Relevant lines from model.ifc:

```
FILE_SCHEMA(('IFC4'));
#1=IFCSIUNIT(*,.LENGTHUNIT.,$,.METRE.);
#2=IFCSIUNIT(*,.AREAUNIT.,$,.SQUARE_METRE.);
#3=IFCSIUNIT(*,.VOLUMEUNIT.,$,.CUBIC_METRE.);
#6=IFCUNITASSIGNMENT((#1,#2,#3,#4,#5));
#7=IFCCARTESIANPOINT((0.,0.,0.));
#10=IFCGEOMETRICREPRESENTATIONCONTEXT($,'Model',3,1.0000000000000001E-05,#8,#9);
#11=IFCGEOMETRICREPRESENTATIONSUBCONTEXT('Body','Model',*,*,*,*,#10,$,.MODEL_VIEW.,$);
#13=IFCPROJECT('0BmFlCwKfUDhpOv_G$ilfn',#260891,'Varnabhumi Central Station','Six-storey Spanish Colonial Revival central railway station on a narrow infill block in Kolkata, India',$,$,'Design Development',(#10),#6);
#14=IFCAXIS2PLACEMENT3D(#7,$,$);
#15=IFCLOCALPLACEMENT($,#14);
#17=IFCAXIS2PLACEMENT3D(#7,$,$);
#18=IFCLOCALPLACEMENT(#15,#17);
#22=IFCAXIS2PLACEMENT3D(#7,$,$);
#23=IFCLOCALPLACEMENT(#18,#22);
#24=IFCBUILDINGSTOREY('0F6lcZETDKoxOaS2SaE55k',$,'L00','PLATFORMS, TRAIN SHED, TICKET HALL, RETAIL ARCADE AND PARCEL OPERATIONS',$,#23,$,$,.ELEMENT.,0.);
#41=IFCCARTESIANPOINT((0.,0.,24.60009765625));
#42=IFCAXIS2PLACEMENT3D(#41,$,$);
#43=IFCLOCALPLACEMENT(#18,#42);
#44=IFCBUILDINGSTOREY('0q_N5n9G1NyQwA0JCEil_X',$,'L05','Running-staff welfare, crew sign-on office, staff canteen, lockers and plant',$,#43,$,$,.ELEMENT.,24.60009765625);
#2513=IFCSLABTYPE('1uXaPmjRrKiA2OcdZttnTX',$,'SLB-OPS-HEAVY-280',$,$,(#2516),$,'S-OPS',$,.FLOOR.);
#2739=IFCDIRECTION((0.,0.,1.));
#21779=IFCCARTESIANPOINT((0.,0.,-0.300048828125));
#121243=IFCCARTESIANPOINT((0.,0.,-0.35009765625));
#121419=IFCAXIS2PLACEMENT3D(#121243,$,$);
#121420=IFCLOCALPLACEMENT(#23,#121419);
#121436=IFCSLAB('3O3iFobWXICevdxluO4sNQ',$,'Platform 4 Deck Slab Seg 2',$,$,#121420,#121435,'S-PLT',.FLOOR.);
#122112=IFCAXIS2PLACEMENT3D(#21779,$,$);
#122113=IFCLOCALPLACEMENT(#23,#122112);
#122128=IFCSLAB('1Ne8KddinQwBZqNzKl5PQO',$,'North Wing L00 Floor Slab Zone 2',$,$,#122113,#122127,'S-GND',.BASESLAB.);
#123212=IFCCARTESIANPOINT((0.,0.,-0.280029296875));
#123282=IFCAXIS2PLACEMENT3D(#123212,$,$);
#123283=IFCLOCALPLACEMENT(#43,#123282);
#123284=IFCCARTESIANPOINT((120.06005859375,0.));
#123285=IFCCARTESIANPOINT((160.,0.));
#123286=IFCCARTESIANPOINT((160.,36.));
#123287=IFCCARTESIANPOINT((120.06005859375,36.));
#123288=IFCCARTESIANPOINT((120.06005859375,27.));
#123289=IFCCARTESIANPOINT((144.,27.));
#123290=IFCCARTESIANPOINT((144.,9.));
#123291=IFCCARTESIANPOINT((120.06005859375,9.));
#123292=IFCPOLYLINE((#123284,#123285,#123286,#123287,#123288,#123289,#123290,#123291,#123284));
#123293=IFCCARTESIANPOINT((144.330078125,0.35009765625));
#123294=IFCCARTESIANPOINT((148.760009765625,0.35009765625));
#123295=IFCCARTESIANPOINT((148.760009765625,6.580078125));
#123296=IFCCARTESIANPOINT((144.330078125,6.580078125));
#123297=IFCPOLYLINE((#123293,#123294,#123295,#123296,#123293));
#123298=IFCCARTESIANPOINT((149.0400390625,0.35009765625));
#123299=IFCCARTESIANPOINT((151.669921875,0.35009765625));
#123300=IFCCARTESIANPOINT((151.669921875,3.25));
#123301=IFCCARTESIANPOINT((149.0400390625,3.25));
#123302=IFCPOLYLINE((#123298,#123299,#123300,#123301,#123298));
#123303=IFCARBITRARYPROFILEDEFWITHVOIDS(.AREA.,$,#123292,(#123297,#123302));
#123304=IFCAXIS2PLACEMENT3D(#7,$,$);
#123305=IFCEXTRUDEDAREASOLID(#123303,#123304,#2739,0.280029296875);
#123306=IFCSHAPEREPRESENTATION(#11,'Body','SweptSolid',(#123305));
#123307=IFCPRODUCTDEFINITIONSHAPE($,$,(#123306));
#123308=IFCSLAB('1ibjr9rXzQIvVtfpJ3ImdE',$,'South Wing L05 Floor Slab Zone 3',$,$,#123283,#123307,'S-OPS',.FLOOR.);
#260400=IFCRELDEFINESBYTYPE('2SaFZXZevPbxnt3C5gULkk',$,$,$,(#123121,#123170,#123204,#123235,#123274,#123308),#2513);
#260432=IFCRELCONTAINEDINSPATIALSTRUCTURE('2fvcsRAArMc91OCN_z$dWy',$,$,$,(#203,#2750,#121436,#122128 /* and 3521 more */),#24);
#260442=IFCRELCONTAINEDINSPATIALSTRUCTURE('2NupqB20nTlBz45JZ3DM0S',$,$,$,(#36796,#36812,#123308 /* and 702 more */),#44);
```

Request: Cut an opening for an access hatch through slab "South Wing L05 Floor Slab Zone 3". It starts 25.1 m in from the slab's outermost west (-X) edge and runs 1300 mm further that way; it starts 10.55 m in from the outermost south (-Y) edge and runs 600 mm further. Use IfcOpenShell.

```python
import numpy as np
import ifcopenshell
import ifcopenshell.api.feature
import ifcopenshell.api.geometry
import ifcopenshell.api.root
import ifcopenshell.geom
import ifcopenshell.util.placement
import ifcopenshell.util.representation
import ifcopenshell.util.shape
import ifcopenshell.util.unit

model = ifcopenshell.open("model.ifc")
unit_scale = ifcopenshell.util.unit.calculate_unit_scale(model)
settings = ifcopenshell.geom.settings()


def volume(element):
    """Net volume in cubic metres, openings subtracted."""
    shape = ifcopenshell.geom.create_shape(settings, element)
    return ifcopenshell.util.shape.get_volume(shape.geometry)


slab = model.by_guid("1ibjr9rXzQIvVtfpJ3ImdE")
before = volume(slab)

# Extent in the slab's own axes, in metres. The edges named are its -X and -Y sides.
slab_shape = ifcopenshell.geom.create_shape(settings, slab)
vertices = ifcopenshell.util.shape.get_vertices(slab_shape.geometry)
x_min, y_min, bottom = vertices.min(axis=0)
top = vertices[:, 2].max()

opening = ifcopenshell.api.root.create_entity(model, ifc_class="IfcOpeningElement", name="Access hatch opening", predefined_type="OPENING")
context = ifcopenshell.util.representation.get_context(model, "Model", "Body", "MODEL_VIEW")
width, depth = 1.3, 0.6
outline = [(0.0, 0.0), (width, 0.0), (width, depth), (0.0, depth), (0.0, 0.0)]
# Overshoot both faces by 50 mm so the cut is clean.
shape = ifcopenshell.api.geometry.add_slab_representation(
    model, context=context, depth=top - bottom + 0.1, polyline=outline
)
ifcopenshell.api.geometry.assign_representation(model, product=opening, representation=shape)

matrix = ifcopenshell.util.placement.get_local_placement(slab.ObjectPlacement)
matrix[:, 3] = matrix @ np.append(np.array([x_min + 25.1, y_min + 10.55, bottom - 0.05]) / unit_scale, 1.0)
ifcopenshell.api.geometry.edit_object_placement(model, product=opening, matrix=matrix, is_si=False)
ifcopenshell.api.feature.add_feature(model, feature=opening, element=slab)

after = volume(slab)

print(f"slab volume {before:.3f} -> {after:.3f} m3")

model.write("model_edited.ifc")
```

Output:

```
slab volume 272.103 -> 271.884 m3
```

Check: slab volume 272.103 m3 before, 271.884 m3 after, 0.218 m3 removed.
